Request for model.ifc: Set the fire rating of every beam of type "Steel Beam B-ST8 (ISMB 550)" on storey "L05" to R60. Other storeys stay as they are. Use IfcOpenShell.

First a look at what the model holds.

```python
import ifcopenshell
import ifcopenshell.util.element

model = ifcopenshell.open("model.ifc")
print(model.schema)
storey = next(s for s in model.by_type("IfcBuildingStorey") if s.Name == "L05")
beams = [e for e in ifcopenshell.util.element.get_decomposition(storey) if e.is_a("IfcBeam")]
seen = {}
for e in beams:
    element_type = ifcopenshell.util.element.get_type(e)
    key = (element_type.Name if element_type != e and element_type else None, ifcopenshell.util.element.get_pset(e, "Pset_BeamCommon", "FireRating"))
    seen[key] = seen.get(key, 0) + 1
for (name, value), count in sorted(seen.items(), key=str):
    print(count, "x", name, "|", value)
```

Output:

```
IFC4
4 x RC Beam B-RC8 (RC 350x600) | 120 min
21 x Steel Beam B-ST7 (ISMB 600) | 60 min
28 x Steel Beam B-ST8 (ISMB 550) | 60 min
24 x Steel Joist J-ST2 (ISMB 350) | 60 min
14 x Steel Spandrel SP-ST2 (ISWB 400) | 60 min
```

```python
import ifcopenshell
import ifcopenshell.api.pset
import ifcopenshell.util.element

model = ifcopenshell.open("model.ifc")

storey = next(s for s in model.by_type("IfcBuildingStorey") if s.Name == "L05")
beams = [e for e in ifcopenshell.util.element.get_decomposition(storey) if e.is_a("IfcBeam")]

count = 0
for e in beams:
    element_type = ifcopenshell.util.element.get_type(e)
    if element_type in (None, e) or element_type.Name != "Steel Beam B-ST8 (ISMB 550)":
        continue
    # add_pset returns the element's existing set when there is one.
    pset = ifcopenshell.api.pset.add_pset(model, product=e, name="Pset_BeamCommon")
    ifcopenshell.api.pset.edit_pset(model, pset=pset, properties={"FireRating": "R60"})
    count += 1

print(count, "beams updated")

model.write("model_updated.ifc")
```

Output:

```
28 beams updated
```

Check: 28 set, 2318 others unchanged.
